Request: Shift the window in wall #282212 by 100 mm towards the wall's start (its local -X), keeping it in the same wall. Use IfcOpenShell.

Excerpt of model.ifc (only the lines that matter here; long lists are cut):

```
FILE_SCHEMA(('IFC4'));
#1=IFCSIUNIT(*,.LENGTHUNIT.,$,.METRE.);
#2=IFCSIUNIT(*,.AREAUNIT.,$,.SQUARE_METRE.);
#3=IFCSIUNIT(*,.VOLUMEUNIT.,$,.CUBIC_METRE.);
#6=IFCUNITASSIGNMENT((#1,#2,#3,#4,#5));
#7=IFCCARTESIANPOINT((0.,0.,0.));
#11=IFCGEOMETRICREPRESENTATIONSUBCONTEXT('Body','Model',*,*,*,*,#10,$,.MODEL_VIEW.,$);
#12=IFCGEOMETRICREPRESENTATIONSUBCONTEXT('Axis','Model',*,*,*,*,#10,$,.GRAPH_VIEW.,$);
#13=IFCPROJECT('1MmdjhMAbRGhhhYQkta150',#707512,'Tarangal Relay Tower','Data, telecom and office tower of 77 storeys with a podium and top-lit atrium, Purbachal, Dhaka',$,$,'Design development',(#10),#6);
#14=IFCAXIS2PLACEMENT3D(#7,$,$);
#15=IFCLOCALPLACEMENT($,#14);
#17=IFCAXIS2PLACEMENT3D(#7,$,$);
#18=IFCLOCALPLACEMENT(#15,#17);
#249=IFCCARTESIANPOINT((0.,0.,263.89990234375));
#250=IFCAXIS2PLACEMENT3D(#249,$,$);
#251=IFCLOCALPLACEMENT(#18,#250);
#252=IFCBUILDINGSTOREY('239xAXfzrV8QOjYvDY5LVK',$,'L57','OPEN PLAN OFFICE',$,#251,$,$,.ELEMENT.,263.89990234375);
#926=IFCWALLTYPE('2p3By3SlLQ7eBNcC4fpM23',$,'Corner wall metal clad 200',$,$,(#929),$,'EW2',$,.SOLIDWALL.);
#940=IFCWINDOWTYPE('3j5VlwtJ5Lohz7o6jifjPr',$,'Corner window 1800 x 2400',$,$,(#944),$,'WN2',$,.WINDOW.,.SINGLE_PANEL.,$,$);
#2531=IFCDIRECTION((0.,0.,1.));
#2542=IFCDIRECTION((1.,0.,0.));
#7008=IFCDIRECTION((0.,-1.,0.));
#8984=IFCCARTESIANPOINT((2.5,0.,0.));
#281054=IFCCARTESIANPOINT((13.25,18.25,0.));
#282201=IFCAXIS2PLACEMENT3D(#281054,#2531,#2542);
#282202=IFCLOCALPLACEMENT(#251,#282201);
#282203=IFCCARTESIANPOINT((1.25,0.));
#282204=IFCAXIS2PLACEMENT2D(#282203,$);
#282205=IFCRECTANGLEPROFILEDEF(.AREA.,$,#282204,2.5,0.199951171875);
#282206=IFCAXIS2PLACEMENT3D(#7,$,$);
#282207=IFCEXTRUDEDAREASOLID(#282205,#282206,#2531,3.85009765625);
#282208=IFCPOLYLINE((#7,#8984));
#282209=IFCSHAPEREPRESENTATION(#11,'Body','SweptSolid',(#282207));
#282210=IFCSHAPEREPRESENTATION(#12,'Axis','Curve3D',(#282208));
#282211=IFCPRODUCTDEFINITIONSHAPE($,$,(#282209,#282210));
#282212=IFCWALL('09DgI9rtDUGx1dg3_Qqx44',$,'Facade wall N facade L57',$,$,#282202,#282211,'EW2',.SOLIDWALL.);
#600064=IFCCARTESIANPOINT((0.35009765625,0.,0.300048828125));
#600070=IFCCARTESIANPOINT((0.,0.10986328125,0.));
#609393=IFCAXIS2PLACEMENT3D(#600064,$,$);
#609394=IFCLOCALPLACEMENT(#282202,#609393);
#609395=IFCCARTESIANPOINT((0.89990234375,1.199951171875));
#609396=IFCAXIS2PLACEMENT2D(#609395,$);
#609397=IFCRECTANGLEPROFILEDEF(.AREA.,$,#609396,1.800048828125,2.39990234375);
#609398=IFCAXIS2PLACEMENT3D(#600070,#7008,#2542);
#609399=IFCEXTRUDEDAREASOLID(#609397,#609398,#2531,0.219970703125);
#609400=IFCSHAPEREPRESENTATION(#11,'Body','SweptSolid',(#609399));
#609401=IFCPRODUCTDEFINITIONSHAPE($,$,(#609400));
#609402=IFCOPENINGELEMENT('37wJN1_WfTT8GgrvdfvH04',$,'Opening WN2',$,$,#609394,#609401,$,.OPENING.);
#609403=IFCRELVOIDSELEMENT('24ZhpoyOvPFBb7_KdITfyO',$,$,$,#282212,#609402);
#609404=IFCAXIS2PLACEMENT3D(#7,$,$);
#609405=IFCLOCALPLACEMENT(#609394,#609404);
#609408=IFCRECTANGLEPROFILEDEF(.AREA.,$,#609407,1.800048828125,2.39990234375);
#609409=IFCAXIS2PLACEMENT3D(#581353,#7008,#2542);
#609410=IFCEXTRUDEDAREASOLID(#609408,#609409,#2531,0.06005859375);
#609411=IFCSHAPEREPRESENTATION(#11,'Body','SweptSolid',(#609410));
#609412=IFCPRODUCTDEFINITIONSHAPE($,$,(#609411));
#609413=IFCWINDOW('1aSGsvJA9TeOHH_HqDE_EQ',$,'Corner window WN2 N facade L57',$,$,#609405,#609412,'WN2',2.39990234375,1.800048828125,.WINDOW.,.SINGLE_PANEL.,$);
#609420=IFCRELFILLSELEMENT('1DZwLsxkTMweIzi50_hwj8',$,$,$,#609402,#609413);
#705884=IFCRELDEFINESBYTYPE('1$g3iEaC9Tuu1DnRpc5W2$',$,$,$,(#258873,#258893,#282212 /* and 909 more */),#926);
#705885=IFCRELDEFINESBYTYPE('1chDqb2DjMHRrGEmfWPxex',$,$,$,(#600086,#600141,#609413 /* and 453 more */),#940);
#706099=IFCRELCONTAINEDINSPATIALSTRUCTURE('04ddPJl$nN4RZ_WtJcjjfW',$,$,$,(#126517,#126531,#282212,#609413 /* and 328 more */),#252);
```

```python
import ifcopenshell
import ifcopenshell.api.geometry
import ifcopenshell.util.placement
import ifcopenshell.util.unit

model = ifcopenshell.open("model.ifc")
unit_scale = ifcopenshell.util.unit.calculate_unit_scale(model)

window = model.by_id(609413)
opening = window.FillsVoids[0].RelatingOpeningElement
wall = opening.VoidsElements[0].RelatingBuildingElement

wall_matrix = ifcopenshell.util.placement.get_local_placement(wall.ObjectPlacement)
shift = wall_matrix[:3, 0] * -0.1 / unit_scale
before = ifcopenshell.util.placement.get_local_placement(window.ObjectPlacement)[:3, 3].copy()

# The window is placed relative to its opening, so it follows when the opening moves.
matrix = ifcopenshell.util.placement.get_local_placement(opening.ObjectPlacement)
matrix[:3, 3] += shift
ifcopenshell.api.geometry.edit_object_placement(
    model, product=opening, matrix=matrix, is_si=False, should_transform_children=True
)

after = ifcopenshell.util.placement.get_local_placement(window.ObjectPlacement)[:3, 3]
print("window moved by", (after - before).round(3) + 0.0)

model.write("model_rev.ifc")
```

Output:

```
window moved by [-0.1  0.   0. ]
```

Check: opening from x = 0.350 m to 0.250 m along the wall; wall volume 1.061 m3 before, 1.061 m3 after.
